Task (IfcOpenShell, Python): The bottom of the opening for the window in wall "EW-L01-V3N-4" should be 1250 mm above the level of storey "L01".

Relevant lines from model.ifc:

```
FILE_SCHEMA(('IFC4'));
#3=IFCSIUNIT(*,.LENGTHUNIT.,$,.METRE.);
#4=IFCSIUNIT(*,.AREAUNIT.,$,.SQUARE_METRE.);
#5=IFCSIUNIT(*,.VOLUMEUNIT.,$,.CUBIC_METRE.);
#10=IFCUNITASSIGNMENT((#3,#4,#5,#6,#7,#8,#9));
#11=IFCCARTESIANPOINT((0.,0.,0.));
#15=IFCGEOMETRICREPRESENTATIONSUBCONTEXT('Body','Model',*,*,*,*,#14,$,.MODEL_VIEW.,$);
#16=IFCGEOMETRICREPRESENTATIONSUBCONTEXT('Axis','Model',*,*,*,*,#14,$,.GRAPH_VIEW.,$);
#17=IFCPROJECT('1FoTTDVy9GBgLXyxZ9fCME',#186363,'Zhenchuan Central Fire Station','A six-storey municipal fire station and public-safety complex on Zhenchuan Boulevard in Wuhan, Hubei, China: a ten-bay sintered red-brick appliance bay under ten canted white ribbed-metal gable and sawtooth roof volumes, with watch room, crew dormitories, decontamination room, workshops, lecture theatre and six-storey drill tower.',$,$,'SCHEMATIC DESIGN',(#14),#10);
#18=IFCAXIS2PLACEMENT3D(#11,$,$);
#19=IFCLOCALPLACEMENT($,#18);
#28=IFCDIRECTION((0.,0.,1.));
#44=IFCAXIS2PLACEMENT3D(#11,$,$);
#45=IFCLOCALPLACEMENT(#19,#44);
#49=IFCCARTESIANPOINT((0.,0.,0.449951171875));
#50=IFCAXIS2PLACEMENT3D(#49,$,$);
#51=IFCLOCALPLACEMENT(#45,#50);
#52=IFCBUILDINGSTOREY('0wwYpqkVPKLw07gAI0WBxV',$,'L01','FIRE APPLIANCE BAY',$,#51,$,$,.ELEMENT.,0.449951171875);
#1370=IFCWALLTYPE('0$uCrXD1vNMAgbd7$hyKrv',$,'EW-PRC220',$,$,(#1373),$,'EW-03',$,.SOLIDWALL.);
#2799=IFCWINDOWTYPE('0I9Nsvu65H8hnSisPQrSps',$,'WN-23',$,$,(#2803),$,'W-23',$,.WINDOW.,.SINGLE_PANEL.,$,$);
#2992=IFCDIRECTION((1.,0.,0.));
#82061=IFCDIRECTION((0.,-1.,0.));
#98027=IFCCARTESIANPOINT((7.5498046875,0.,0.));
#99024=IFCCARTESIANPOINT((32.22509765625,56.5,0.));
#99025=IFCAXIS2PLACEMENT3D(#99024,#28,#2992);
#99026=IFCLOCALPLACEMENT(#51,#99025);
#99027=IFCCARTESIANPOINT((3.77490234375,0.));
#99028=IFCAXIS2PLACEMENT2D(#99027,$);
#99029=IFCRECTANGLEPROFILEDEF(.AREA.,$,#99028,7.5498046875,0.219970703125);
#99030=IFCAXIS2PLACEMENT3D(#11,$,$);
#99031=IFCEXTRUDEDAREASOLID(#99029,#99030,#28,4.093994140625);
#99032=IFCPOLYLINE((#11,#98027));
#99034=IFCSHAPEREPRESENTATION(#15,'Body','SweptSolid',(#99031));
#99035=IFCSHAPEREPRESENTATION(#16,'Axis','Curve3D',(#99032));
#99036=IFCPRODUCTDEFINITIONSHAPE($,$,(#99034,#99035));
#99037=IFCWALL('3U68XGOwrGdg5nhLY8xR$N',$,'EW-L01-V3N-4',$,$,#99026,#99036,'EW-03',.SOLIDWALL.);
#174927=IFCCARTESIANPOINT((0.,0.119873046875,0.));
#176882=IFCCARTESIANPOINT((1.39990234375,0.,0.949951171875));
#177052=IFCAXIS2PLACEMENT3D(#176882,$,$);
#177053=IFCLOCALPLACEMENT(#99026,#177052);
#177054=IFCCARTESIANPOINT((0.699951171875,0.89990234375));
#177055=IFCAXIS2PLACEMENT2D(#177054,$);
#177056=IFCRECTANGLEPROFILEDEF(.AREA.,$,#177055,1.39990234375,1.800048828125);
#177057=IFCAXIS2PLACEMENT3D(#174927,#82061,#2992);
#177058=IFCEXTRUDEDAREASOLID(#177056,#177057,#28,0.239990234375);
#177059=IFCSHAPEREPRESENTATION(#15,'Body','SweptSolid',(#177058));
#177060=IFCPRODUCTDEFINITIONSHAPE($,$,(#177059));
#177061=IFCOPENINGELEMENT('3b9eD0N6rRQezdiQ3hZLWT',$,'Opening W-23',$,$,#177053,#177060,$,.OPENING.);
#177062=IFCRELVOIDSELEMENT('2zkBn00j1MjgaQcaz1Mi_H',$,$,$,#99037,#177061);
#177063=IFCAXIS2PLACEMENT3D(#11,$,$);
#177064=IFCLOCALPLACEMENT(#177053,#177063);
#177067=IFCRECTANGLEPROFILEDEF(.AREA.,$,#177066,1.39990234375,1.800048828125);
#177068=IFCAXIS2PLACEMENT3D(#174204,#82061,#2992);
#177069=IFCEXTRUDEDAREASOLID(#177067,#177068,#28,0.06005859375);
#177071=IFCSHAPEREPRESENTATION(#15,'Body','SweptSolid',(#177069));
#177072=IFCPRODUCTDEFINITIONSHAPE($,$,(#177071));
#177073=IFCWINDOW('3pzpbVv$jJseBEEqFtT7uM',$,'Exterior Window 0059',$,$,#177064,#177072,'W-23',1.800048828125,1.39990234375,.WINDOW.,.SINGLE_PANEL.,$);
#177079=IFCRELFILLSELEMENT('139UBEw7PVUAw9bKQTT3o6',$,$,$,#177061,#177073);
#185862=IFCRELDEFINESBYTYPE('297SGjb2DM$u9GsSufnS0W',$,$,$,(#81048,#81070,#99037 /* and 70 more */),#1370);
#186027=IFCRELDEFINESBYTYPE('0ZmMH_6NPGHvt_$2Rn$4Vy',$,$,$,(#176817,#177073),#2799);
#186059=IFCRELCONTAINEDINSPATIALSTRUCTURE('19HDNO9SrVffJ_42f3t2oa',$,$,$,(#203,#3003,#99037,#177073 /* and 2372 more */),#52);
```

```python
import numpy as np
import ifcopenshell
import ifcopenshell.api.geometry
import ifcopenshell.geom
import ifcopenshell.util.element
import ifcopenshell.util.placement
import ifcopenshell.util.shape
import ifcopenshell.util.unit

model = ifcopenshell.open("model.ifc")
unit_scale = ifcopenshell.util.unit.calculate_unit_scale(model)

window = model.by_id(177073)
opening = window.FillsVoids[0].RelatingOpeningElement
storey = ifcopenshell.util.element.get_container(window, ifc_class="IfcBuildingStorey")
level = ifcopenshell.util.placement.get_local_placement(storey.ObjectPlacement)[2, 3]

# The opening's origin need not be at the sill, so measure its lowest point.
shape = ifcopenshell.geom.create_shape(ifcopenshell.geom.settings(), opening)
bottom = ifcopenshell.util.shape.get_shape_bottom_elevation(shape, shape.geometry) / unit_scale
dz = level + 1.25 / unit_scale - bottom

shift = np.array([0.0, 0.0, dz])
# The window is placed relative to its opening, so it follows when the opening moves.
matrix = ifcopenshell.util.placement.get_local_placement(opening.ObjectPlacement)
matrix[:3, 3] += shift
ifcopenshell.api.geometry.edit_object_placement(
    model, product=opening, matrix=matrix, is_si=False, should_transform_children=True
)

print(f"moved by {dz * unit_scale:+.3f} m")

model.write("model_v2.ifc")
```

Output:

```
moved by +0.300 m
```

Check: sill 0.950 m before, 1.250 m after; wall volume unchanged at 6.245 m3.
